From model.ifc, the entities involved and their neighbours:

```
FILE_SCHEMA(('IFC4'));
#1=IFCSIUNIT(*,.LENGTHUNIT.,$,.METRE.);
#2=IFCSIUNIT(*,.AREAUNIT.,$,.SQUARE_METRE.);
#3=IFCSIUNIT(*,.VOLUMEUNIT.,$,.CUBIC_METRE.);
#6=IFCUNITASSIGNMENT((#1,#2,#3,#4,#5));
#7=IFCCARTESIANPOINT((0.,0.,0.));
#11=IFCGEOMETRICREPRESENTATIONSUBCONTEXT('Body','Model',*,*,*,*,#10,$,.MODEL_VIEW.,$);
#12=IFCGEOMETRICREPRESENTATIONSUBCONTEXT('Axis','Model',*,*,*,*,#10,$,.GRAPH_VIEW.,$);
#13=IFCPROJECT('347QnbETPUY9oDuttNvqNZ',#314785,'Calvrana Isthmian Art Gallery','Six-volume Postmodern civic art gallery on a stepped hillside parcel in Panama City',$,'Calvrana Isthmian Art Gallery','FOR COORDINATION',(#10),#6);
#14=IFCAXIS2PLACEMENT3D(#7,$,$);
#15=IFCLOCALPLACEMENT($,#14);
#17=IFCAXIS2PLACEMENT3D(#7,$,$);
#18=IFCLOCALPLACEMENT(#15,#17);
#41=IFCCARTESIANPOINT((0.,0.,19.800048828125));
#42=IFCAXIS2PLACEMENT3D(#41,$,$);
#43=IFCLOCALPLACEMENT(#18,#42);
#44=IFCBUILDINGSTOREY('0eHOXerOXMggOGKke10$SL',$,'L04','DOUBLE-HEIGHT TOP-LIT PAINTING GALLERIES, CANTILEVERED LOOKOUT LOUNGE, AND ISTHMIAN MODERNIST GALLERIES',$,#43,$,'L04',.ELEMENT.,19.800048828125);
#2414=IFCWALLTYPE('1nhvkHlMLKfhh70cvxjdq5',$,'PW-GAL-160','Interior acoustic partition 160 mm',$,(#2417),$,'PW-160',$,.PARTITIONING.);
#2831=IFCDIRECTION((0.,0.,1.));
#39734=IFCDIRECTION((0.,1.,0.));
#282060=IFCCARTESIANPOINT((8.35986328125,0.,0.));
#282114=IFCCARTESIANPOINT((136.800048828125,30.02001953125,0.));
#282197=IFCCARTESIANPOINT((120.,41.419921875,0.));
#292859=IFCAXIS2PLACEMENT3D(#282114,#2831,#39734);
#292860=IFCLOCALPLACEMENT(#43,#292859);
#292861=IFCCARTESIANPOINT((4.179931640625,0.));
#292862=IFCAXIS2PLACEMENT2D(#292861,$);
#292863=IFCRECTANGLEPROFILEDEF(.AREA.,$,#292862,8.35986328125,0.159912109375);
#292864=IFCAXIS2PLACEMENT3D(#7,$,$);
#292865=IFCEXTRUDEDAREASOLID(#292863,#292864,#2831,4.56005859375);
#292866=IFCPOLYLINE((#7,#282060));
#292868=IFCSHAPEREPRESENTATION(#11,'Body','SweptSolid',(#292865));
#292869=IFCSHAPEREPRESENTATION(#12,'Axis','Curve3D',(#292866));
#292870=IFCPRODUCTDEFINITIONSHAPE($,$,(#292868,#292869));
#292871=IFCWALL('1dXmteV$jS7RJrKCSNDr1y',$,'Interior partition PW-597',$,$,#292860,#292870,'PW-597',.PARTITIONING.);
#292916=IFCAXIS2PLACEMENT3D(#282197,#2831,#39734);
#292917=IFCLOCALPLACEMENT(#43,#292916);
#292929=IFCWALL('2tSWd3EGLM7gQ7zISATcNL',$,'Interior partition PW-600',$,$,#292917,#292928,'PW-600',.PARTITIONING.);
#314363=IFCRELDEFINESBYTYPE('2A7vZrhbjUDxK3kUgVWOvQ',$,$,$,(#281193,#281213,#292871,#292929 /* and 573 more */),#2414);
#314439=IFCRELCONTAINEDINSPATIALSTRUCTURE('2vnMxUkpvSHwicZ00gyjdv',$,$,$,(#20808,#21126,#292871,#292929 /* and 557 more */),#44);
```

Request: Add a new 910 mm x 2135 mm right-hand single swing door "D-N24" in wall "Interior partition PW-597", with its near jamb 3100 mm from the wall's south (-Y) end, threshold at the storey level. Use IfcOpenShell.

```python
import numpy as np
import ifcopenshell
import ifcopenshell.api.feature
import ifcopenshell.api.geometry
import ifcopenshell.api.root
import ifcopenshell.api.spatial
import ifcopenshell.geom
import ifcopenshell.util.element
import ifcopenshell.util.placement
import ifcopenshell.util.representation
import ifcopenshell.util.shape
import ifcopenshell.util.unit

model = ifcopenshell.open("model.ifc")
unit_scale = ifcopenshell.util.unit.calculate_unit_scale(model)
settings = ifcopenshell.geom.settings()


def volume(element):
    """Net volume in cubic metres, openings subtracted."""
    shape = ifcopenshell.geom.create_shape(settings, element)
    return ifcopenshell.util.shape.get_volume(shape.geometry)


wall = model.by_guid("1dXmteV$jS7RJrKCSNDr1y")
storey = ifcopenshell.util.element.get_container(wall, ifc_class="IfcBuildingStorey")
context = ifcopenshell.util.representation.get_context(model, "Model", "Body", "MODEL_VIEW")
before = volume(wall)

width, height, from_end, sill = 0.91, 2.135, 3.1, 0.0  # metres

# The wall runs along its own X axis, and the end named is its -X end.
wall_shape = ifcopenshell.geom.create_shape(settings, wall)
x, y, z = ifcopenshell.util.shape.get_vertices(wall_shape.geometry).T
start = x.min() + from_end
face, thickness = float(y.min()), float(y.max() - y.min())
wall_matrix = ifcopenshell.util.placement.get_local_placement(wall.ObjectPlacement)
level = ifcopenshell.util.placement.get_local_placement(storey.ObjectPlacement)[2, 3]


def in_wall(x, y):
    """Placement at x, y metres in the wall's axes, at sill height."""
    matrix = wall_matrix.copy()
    matrix[:, 3] = wall_matrix @ np.array([x / unit_scale, y / unit_scale, 0.0, 1.0])
    matrix[2, 3] = level + sill / unit_scale
    return matrix


# Opening: a box that overshoots both wall faces by 50 mm.
opening = ifcopenshell.api.root.create_entity(model, ifc_class="IfcOpeningElement", predefined_type="OPENING")
box = ifcopenshell.api.geometry.add_wall_representation(
    model, context=context, length=width, height=height, thickness=thickness + 0.1
)
ifcopenshell.api.geometry.assign_representation(model, product=opening, representation=box)
ifcopenshell.api.geometry.edit_object_placement(model, product=opening, matrix=in_wall(start, face - 0.05), is_si=False)
ifcopenshell.api.feature.add_feature(model, feature=opening, element=wall)

door = ifcopenshell.api.root.create_entity(model, ifc_class="IfcDoor", name="D-N24", predefined_type="DOOR")
door.OverallWidth, door.OverallHeight = width / unit_scale, height / unit_scale
door.OperationType = "SINGLE_SWING_RIGHT"
body = ifcopenshell.api.geometry.add_door_representation(
    model,
    context=context,
    overall_width=door.OverallWidth,
    overall_height=door.OverallHeight,
    operation_type="SINGLE_SWING_RIGHT",
    lining_properties={"LiningDepth": thickness / unit_scale, "ThresholdDepth": thickness / unit_scale},
)
ifcopenshell.api.geometry.assign_representation(model, product=door, representation=body)
ifcopenshell.api.spatial.assign_container(model, products=[door], relating_structure=storey)
ifcopenshell.api.feature.add_filling(model, opening=opening, element=door)

# The lining spans the wall, so the door starts at the wall face.
ifcopenshell.api.geometry.edit_object_placement(model, product=door, matrix=in_wall(start, face), is_si=False)

after = volume(wall)

print(f"wall volume {before:.3f} -> {after:.3f} m3")

model.write("model_rev.ifc")
```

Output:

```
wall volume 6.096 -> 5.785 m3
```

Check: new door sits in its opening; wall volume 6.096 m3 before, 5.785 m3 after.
